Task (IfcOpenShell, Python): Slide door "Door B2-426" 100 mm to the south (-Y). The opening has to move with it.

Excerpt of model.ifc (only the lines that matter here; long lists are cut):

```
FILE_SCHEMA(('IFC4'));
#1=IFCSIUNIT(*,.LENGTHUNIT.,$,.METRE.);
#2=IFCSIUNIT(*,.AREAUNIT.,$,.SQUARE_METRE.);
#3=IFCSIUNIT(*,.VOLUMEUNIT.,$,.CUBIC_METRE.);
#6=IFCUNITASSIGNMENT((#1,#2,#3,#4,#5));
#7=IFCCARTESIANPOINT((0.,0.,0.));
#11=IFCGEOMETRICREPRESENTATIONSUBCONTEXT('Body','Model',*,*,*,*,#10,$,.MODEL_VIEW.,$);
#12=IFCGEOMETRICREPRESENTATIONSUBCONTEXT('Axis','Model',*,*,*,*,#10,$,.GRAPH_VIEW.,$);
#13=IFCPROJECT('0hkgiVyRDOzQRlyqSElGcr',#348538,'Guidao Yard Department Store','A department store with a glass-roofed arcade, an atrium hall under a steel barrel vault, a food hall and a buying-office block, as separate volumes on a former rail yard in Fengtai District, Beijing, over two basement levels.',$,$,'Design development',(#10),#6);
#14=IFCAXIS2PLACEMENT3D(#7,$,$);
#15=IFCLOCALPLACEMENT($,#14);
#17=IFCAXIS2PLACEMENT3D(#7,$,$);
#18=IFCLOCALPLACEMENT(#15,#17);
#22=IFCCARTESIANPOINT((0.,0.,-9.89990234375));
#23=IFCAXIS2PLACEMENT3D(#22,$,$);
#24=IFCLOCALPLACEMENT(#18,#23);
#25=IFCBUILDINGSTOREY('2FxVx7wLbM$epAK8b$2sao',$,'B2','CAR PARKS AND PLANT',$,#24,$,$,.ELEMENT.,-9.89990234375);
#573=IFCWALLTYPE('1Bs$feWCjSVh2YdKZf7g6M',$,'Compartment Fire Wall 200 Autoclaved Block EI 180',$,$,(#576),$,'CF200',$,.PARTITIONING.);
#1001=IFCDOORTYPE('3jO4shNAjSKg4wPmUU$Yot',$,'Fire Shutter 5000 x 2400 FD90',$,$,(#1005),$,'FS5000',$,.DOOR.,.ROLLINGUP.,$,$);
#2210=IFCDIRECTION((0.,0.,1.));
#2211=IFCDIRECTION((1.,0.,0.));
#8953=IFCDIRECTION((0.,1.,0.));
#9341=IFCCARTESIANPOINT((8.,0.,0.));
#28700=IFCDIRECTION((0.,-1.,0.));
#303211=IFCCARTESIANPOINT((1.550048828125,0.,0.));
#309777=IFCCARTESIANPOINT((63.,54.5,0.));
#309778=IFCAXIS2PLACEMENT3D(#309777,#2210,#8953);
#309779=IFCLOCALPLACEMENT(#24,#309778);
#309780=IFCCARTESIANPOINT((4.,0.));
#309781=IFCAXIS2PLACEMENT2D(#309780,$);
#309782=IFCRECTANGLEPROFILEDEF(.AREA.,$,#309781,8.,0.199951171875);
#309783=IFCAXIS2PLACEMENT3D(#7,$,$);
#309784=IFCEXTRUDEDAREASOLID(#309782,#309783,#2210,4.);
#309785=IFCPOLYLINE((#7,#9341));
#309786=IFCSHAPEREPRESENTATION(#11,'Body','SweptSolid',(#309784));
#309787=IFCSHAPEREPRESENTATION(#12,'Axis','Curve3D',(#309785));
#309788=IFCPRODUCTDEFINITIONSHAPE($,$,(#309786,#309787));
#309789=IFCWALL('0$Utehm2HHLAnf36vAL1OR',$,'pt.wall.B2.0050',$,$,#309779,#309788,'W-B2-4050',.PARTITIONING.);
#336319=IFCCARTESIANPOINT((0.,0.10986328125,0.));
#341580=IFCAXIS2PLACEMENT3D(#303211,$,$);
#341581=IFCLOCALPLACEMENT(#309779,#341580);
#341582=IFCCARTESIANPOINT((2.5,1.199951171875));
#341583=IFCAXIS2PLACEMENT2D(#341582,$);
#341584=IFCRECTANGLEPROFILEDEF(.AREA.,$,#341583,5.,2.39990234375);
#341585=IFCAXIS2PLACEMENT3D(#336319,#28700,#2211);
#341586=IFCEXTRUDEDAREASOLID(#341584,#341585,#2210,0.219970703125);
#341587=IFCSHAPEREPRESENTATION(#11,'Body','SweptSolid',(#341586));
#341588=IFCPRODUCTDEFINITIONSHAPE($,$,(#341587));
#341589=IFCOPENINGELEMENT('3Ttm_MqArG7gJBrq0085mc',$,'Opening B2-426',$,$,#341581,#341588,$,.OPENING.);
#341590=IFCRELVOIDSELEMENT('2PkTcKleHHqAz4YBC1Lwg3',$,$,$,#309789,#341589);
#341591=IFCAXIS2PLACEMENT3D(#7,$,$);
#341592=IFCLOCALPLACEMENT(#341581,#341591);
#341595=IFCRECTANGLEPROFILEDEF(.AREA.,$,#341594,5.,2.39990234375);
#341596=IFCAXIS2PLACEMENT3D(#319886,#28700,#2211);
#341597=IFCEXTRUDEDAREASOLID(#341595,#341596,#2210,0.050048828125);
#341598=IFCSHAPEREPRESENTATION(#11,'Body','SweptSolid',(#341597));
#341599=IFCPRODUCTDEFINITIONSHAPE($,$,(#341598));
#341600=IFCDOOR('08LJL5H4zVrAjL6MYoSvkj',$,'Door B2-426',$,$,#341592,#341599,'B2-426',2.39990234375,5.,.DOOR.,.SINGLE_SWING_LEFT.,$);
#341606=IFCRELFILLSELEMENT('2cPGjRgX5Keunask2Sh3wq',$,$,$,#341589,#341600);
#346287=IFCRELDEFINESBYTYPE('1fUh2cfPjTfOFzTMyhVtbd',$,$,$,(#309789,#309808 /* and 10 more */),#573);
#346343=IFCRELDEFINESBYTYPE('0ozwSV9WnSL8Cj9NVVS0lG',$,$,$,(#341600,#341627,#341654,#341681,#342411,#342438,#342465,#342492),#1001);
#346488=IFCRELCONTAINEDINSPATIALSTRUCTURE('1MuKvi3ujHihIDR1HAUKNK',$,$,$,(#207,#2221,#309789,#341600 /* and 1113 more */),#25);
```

```python
import ifcopenshell
import ifcopenshell.api.geometry
import ifcopenshell.util.placement
import ifcopenshell.util.unit

model = ifcopenshell.open("model.ifc")
unit_scale = ifcopenshell.util.unit.calculate_unit_scale(model)

door = model.by_guid("08LJL5H4zVrAjL6MYoSvkj")
opening = door.FillsVoids[0].RelatingOpeningElement
wall = opening.VoidsElements[0].RelatingBuildingElement

wall_matrix = ifcopenshell.util.placement.get_local_placement(wall.ObjectPlacement)
shift = wall_matrix[:3, 0] * -0.1 / unit_scale
before = ifcopenshell.util.placement.get_local_placement(door.ObjectPlacement)[:3, 3].copy()

# The door is placed relative to its opening, so it follows when the opening moves.
matrix = ifcopenshell.util.placement.get_local_placement(opening.ObjectPlacement)
matrix[:3, 3] += shift
ifcopenshell.api.geometry.edit_object_placement(
    model, product=opening, matrix=matrix, is_si=False, should_transform_children=True
)

after = ifcopenshell.util.placement.get_local_placement(door.ObjectPlacement)[:3, 3]
print("door moved by", (after - before).round(3) + 0.0)

model.write("model-out.ifc")
```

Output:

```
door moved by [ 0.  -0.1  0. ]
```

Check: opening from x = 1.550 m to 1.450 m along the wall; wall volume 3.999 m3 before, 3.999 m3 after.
